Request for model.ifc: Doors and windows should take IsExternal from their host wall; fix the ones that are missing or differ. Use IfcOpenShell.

First a look at what the model holds.

```python
import ifcopenshell
import ifcopenshell.util.element

model = ifcopenshell.open("model.ifc")
print(model.schema)
seen = {}
for e in model.by_type("IfcDoor") + model.by_type("IfcWindow"):
    if not e.FillsVoids:
        continue
    host = e.FillsVoids[0].RelatingOpeningElement.VoidsElements[0].RelatingBuildingElement
    own = ifcopenshell.util.element.get_pset(e, f"Pset_{e.is_a()[3:].removesuffix('StandardCase')}Common", "IsExternal")
    wall = ifcopenshell.util.element.get_pset(host, "Pset_WallCommon", "IsExternal")
    seen[e.is_a(), own, wall] = seen.get((e.is_a(), own, wall), 0) + 1
for (cls, own, wall), count in sorted(seen.items(), key=str):
    print(count, cls, "IsExternal:", own, "| host wall:", wall)
```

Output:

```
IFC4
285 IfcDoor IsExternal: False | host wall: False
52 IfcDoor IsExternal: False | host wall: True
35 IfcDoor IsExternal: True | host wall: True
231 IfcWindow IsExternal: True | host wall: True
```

```python
import ifcopenshell
import ifcopenshell.api.pset
import ifcopenshell.util.element

model = ifcopenshell.open("model.ifc")

count = 0
for ifc_class, pset_name in (("IfcDoor", "Pset_DoorCommon"), ("IfcWindow", "Pset_WindowCommon")):
    for e in model.by_type(ifc_class):
        if not e.FillsVoids:
            continue
        host = e.FillsVoids[0].RelatingOpeningElement.VoidsElements[0].RelatingBuildingElement
        external = ifcopenshell.util.element.get_pset(host, "Pset_WallCommon", "IsExternal")
        if external is None or ifcopenshell.util.element.get_pset(e, pset_name, "IsExternal") == external:
            continue
        pset = ifcopenshell.api.pset.add_pset(model, product=e, name=pset_name)
        ifcopenshell.api.pset.edit_pset(model, pset=pset, properties={"IsExternal": external})
        count += 1

print(count, "updated")

model.write("model_updated.ifc")
```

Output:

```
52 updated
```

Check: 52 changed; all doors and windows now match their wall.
